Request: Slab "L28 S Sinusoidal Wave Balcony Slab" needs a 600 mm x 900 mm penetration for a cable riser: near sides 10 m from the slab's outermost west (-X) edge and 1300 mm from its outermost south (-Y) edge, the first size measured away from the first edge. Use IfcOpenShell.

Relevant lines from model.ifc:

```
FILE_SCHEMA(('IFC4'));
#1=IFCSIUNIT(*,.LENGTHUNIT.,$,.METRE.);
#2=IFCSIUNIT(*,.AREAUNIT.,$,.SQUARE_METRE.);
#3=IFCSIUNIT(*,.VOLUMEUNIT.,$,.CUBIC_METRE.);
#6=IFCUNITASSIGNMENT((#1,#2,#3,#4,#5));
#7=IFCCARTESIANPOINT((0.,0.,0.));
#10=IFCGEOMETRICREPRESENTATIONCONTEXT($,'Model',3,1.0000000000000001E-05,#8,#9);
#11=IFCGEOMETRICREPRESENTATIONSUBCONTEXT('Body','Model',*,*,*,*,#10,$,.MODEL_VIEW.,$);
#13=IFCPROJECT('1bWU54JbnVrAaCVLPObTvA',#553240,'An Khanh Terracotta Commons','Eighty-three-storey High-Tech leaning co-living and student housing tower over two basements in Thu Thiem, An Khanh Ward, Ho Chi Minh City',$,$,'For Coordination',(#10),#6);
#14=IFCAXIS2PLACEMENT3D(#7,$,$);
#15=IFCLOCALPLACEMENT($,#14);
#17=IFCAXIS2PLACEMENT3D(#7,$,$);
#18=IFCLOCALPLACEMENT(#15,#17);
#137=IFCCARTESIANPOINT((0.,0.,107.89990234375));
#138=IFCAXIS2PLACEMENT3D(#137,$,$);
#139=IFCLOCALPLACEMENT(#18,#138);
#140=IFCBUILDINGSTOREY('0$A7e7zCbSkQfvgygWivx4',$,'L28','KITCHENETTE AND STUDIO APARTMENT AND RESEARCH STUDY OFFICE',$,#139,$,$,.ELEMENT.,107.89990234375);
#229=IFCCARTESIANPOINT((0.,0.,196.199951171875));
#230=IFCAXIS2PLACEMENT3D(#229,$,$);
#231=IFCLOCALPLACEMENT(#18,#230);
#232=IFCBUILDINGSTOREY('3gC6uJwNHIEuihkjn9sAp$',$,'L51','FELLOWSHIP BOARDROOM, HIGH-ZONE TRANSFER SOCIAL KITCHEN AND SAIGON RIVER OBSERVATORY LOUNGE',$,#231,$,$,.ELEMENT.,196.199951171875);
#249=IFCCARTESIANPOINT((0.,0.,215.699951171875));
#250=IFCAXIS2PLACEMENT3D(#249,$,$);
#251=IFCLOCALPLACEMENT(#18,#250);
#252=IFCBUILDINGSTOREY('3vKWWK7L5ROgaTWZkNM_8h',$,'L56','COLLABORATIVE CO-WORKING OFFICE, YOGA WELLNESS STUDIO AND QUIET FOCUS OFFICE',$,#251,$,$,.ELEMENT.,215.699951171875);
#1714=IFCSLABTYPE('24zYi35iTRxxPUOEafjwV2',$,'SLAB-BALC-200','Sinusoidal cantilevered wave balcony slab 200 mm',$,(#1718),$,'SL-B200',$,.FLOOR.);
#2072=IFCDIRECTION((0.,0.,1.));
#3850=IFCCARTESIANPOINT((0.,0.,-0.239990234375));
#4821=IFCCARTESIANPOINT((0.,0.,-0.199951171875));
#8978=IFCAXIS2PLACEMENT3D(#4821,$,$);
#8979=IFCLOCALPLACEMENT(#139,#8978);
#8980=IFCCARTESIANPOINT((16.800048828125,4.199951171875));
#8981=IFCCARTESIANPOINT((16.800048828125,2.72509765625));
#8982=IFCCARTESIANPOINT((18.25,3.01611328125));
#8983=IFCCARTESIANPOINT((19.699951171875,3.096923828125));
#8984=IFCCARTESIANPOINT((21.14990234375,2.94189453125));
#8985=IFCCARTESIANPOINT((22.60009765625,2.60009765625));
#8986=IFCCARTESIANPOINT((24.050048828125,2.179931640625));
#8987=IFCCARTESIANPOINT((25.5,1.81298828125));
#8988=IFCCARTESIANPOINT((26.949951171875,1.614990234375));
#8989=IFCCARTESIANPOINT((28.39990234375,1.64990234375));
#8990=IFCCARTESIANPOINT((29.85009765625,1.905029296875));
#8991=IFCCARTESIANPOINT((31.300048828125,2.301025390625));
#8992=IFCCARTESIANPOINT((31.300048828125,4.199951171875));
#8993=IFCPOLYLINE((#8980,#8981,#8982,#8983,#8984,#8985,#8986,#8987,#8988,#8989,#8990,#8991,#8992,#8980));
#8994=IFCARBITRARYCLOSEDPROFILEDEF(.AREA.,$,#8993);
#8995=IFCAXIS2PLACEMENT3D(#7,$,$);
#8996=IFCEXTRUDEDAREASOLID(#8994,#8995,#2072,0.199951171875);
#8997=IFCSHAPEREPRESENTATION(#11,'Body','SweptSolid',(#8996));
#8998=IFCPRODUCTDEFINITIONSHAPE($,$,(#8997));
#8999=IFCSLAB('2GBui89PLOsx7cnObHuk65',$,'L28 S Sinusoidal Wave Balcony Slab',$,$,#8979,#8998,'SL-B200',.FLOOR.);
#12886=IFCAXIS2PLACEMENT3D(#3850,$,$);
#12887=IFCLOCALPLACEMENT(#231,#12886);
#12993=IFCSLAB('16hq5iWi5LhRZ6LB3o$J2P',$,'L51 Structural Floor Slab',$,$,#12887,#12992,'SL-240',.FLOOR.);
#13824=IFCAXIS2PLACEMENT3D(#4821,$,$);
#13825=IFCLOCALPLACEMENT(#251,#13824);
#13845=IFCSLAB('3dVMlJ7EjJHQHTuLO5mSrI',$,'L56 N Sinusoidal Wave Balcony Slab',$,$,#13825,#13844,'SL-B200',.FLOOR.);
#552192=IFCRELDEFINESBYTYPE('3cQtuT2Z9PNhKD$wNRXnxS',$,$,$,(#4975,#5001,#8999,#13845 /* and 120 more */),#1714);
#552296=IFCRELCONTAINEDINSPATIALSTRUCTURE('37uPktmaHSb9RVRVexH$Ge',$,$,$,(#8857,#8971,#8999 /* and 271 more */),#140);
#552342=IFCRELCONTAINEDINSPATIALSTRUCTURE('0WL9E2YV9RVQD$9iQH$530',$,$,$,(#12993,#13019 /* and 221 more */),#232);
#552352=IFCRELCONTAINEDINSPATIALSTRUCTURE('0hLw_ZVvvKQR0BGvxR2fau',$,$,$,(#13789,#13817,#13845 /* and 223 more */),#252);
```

```python
import numpy as np
import ifcopenshell
import ifcopenshell.api.feature
import ifcopenshell.api.geometry
import ifcopenshell.api.root
import ifcopenshell.geom
import ifcopenshell.util.placement
import ifcopenshell.util.representation
import ifcopenshell.util.shape
import ifcopenshell.util.unit

model = ifcopenshell.open("model.ifc")
unit_scale = ifcopenshell.util.unit.calculate_unit_scale(model)
settings = ifcopenshell.geom.settings()


def volume(element):
    """Net volume in cubic metres, openings subtracted."""
    shape = ifcopenshell.geom.create_shape(settings, element)
    return ifcopenshell.util.shape.get_volume(shape.geometry)


slab = model.by_guid("2GBui89PLOsx7cnObHuk65")
before = volume(slab)

# Extent in the slab's own axes, in metres. The edges named are its -X and -Y sides.
slab_shape = ifcopenshell.geom.create_shape(settings, slab)
vertices = ifcopenshell.util.shape.get_vertices(slab_shape.geometry)
x_min, y_min, bottom = vertices.min(axis=0)
top = vertices[:, 2].max()

opening = ifcopenshell.api.root.create_entity(model, ifc_class="IfcOpeningElement", name="Cable riser opening", predefined_type="OPENING")
context = ifcopenshell.util.representation.get_context(model, "Model", "Body", "MODEL_VIEW")
width, depth = 0.6, 0.9
outline = [(0.0, 0.0), (width, 0.0), (width, depth), (0.0, depth), (0.0, 0.0)]
# Overshoot both faces by 50 mm so the cut is clean.
shape = ifcopenshell.api.geometry.add_slab_representation(
    model, context=context, depth=top - bottom + 0.1, polyline=outline
)
ifcopenshell.api.geometry.assign_representation(model, product=opening, representation=shape)

matrix = ifcopenshell.util.placement.get_local_placement(slab.ObjectPlacement)
matrix[:, 3] = matrix @ np.append(np.array([x_min + 10, y_min + 1.3, bottom - 0.05]) / unit_scale, 1.0)
ifcopenshell.api.geometry.edit_object_placement(model, product=opening, matrix=matrix, is_si=False)
ifcopenshell.api.feature.add_feature(model, feature=opening, element=slab)

after = volume(slab)

print(f"slab volume {before:.3f} -> {after:.3f} m3")

model.write("model_edited.ifc")
```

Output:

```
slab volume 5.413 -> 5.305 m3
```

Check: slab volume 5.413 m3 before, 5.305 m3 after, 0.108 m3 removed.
